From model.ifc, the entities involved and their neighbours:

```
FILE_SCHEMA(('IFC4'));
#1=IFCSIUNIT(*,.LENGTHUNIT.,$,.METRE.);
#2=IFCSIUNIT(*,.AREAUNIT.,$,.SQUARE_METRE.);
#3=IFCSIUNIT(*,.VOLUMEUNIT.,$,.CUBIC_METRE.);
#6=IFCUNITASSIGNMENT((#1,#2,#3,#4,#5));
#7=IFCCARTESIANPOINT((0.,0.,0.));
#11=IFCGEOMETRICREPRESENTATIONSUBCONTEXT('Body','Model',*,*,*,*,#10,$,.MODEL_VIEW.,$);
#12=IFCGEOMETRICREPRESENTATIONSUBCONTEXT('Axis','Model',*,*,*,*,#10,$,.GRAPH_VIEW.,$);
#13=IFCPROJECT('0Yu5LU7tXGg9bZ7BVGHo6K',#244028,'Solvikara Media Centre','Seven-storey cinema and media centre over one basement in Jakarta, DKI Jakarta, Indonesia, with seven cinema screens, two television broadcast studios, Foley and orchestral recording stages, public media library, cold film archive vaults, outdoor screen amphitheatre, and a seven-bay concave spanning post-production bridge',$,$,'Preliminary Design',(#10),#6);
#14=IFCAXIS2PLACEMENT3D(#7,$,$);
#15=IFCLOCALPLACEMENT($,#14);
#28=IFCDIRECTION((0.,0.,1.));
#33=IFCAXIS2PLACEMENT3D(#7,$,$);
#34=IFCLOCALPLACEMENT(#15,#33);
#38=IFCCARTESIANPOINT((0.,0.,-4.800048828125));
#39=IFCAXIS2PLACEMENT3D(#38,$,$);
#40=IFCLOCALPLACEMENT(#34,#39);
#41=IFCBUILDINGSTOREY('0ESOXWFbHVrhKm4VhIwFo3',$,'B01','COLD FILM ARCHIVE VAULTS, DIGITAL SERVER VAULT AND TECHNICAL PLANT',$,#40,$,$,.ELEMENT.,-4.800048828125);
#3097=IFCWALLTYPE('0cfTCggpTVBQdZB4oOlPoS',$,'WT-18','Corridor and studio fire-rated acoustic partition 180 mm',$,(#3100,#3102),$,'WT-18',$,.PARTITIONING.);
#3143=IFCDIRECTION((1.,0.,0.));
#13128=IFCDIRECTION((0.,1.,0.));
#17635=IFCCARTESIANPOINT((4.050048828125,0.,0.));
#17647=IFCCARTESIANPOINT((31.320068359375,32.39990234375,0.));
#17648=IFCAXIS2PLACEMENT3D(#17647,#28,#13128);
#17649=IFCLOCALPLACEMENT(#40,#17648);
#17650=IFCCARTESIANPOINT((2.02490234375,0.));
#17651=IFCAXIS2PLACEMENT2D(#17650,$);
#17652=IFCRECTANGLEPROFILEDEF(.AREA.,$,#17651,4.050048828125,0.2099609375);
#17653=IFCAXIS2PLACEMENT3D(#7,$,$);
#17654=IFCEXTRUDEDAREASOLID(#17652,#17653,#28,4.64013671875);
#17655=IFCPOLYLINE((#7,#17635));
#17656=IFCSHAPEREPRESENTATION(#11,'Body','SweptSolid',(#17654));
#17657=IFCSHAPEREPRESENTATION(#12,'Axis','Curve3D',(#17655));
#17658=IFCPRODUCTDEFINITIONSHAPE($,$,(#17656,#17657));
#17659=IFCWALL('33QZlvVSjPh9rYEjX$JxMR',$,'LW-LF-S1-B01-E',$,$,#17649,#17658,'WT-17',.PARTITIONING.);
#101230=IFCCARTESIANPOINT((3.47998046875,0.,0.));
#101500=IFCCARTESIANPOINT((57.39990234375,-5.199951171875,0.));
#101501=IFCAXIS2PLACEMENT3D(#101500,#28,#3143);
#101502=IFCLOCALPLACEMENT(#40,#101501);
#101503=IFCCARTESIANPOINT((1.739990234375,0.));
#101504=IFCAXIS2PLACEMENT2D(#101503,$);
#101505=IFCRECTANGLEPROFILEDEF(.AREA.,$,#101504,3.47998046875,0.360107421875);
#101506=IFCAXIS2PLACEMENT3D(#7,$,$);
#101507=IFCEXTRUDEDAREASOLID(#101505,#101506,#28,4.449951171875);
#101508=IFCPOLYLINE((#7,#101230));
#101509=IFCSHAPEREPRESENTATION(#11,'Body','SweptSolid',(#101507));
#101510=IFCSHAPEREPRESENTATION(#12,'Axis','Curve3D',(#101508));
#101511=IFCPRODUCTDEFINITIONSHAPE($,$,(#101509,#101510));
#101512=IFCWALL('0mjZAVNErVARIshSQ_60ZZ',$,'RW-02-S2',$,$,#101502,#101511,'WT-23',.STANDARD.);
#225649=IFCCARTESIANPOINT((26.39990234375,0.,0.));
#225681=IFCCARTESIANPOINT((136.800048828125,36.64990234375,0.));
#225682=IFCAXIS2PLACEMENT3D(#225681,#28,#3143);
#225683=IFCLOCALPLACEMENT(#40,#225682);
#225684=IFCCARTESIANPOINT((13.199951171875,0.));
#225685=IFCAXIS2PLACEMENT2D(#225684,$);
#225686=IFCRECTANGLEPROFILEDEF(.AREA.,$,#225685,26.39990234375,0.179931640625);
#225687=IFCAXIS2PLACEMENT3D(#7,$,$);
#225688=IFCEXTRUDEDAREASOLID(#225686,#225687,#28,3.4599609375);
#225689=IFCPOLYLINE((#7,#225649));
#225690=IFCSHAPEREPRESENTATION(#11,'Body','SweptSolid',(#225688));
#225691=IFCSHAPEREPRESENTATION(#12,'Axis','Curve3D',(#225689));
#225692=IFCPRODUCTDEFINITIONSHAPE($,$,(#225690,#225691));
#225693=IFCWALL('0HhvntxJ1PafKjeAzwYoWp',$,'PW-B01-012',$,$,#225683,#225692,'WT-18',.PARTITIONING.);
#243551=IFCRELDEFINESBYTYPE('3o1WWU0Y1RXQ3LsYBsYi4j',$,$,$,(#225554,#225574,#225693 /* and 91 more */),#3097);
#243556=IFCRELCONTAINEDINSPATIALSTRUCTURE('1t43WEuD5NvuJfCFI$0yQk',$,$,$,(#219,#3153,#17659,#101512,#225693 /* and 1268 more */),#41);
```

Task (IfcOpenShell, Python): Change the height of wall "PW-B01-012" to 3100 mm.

```python
import ifcopenshell
import ifcopenshell.geom
import ifcopenshell.util.representation
import ifcopenshell.util.shape
import ifcopenshell.util.unit

model = ifcopenshell.open("model.ifc")
unit_scale = ifcopenshell.util.unit.calculate_unit_scale(model)
settings = ifcopenshell.geom.settings()


def volume(element):
    """Net volume in cubic metres, openings subtracted."""
    shape = ifcopenshell.geom.create_shape(settings, element)
    return ifcopenshell.util.shape.get_volume(shape.geometry)


wall = model.by_id(225693)
before = volume(wall)

body = ifcopenshell.util.representation.get_representation(wall, "Model", "Body")
solid = body.Items[0]
old_height = solid.Depth
solid.Depth = 3.1 / unit_scale
after = volume(wall)

print(f"height {old_height:g} -> {solid.Depth:g}, volume {before:.3f} -> {after:.3f} m3")

model.write("model_rev.ifc")
```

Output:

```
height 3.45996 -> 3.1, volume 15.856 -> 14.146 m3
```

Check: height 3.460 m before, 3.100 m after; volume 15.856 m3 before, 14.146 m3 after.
